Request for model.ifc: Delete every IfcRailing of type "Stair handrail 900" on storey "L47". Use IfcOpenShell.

First a look at what the model holds.

```python
import ifcopenshell
import ifcopenshell.util.element

model = ifcopenshell.open("model.ifc")
print(model.schema)
storey = next(s for s in model.by_type("IfcBuildingStorey") if s.Name == "L47")
railings = [e for e in ifcopenshell.util.element.get_decomposition(storey) if e.is_a("IfcRailing")]
seen = {}
for e in railings:
    element_type = ifcopenshell.util.element.get_type(e)
    name = element_type.Name if element_type not in (None, e) else None
    seen[name] = seen.get(name, 0) + 1
for name, count in sorted(seen.items(), key=str):
    print(count, "x", name)
```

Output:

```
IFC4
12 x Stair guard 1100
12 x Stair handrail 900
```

```python
import ifcopenshell
import ifcopenshell.api.root
import ifcopenshell.util.element

model = ifcopenshell.open("model.ifc")

storey = next(s for s in model.by_type("IfcBuildingStorey") if s.Name == "L47")
railings = [e for e in ifcopenshell.util.element.get_decomposition(storey) if e.is_a("IfcRailing")]
targets = [e for e in railings if (t := ifcopenshell.util.element.get_type(e)) not in (None, e) and t.Name == "Stair handrail 900"]

for e in targets:
    ifcopenshell.api.root.remove_product(model, product=e)
print(len(targets), "removed")

model.write("model_v2.ifc")
```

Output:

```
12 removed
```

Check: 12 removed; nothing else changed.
